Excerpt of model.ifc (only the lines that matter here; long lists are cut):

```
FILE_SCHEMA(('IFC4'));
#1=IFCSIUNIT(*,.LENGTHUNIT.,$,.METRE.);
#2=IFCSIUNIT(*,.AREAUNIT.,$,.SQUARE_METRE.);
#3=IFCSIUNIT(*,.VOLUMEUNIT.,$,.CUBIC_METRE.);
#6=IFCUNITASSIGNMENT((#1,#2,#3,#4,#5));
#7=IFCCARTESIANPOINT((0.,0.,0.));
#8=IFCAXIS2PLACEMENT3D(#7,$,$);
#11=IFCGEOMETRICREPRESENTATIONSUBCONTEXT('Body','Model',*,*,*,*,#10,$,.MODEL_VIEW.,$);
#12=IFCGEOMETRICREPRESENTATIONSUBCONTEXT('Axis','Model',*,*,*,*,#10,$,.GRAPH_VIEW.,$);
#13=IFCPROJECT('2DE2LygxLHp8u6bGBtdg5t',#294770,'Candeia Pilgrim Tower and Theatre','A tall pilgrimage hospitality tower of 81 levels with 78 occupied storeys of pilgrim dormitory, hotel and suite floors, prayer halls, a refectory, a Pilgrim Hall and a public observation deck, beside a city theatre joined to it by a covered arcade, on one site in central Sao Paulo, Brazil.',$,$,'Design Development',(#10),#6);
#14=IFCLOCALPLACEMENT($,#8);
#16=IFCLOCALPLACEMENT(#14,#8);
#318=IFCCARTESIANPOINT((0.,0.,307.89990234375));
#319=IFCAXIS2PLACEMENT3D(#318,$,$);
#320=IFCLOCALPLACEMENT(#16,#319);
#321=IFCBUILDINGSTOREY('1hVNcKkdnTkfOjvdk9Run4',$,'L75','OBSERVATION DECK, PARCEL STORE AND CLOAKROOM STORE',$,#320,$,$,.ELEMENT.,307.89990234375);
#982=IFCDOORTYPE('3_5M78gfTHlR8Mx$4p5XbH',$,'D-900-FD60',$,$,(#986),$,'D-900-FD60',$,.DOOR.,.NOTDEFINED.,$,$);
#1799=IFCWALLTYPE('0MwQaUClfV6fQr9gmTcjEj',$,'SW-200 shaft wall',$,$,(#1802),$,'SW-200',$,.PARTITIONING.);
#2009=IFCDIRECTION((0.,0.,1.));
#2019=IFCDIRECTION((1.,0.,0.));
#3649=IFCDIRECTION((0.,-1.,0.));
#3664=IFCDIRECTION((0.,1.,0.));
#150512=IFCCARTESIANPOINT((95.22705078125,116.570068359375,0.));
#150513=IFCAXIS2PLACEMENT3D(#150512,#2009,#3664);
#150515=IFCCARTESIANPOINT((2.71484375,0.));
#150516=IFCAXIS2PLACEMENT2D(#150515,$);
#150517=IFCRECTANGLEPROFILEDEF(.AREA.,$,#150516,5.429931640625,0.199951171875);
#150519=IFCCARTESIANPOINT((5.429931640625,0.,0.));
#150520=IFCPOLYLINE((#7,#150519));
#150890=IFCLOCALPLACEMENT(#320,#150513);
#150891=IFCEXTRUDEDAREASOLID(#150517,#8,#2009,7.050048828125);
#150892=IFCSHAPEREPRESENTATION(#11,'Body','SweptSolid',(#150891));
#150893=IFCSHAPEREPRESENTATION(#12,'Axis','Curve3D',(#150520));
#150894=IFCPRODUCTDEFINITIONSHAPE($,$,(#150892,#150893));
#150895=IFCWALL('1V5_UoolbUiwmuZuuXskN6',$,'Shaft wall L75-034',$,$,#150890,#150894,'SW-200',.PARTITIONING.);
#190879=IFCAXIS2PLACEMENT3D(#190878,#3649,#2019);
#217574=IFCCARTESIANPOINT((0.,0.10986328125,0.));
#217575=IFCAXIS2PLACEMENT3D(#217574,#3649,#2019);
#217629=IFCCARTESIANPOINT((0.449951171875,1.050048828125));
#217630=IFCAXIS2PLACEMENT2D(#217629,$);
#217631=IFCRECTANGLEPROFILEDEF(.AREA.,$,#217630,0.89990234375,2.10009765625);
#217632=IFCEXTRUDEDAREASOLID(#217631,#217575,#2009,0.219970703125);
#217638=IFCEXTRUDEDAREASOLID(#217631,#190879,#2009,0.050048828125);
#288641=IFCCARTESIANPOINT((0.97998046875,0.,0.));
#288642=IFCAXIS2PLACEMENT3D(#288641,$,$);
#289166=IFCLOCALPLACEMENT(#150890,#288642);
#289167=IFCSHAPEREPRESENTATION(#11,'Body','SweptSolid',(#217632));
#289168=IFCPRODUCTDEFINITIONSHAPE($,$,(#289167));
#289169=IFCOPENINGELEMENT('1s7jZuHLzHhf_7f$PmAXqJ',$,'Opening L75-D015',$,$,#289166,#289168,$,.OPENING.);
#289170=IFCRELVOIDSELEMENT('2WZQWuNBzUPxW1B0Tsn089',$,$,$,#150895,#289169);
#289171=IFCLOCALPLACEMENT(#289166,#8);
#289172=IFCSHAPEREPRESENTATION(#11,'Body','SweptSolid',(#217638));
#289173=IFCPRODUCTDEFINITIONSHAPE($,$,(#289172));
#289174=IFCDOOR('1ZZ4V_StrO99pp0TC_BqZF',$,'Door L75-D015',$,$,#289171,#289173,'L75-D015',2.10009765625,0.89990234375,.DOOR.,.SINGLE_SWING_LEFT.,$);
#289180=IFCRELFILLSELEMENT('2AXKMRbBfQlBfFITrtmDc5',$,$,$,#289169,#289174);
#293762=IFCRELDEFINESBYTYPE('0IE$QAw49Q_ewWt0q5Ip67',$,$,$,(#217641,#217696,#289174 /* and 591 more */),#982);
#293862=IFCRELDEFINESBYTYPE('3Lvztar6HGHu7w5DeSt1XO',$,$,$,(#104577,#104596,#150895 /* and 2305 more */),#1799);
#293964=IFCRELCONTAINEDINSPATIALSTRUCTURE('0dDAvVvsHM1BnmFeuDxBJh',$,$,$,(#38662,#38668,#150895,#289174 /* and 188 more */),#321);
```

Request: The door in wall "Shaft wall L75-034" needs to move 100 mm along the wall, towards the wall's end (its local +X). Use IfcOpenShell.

```python
import ifcopenshell
import ifcopenshell.api.geometry
import ifcopenshell.util.placement
import ifcopenshell.util.unit

model = ifcopenshell.open("model.ifc")
unit_scale = ifcopenshell.util.unit.calculate_unit_scale(model)

door = model.by_guid("1ZZ4V_StrO99pp0TC_BqZF")
opening = door.FillsVoids[0].RelatingOpeningElement
wall = opening.VoidsElements[0].RelatingBuildingElement

wall_matrix = ifcopenshell.util.placement.get_local_placement(wall.ObjectPlacement)
shift = wall_matrix[:3, 0] * 0.1 / unit_scale
before = ifcopenshell.util.placement.get_local_placement(door.ObjectPlacement)[:3, 3].copy()

# The door is placed relative to its opening, so it follows when the opening moves.
matrix = ifcopenshell.util.placement.get_local_placement(opening.ObjectPlacement)
matrix[:3, 3] += shift
ifcopenshell.api.geometry.edit_object_placement(
    model, product=opening, matrix=matrix, is_si=False, should_transform_children=True
)

after = ifcopenshell.util.placement.get_local_placement(door.ObjectPlacement)[:3, 3]
print("door moved by", (after - before).round(3) + 0.0)

model.write("model_v2.ifc")
```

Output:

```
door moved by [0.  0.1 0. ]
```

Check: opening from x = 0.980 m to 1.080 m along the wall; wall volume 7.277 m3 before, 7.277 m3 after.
